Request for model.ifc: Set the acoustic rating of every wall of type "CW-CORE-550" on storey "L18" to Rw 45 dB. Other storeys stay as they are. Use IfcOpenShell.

First a look at what the model holds.

```python
import ifcopenshell
import ifcopenshell.util.element

model = ifcopenshell.open("model.ifc")
print(model.schema)
storey = next(s for s in model.by_type("IfcBuildingStorey") if s.Name == "L18")
walls = [e for e in ifcopenshell.util.element.get_decomposition(storey) if e.is_a("IfcWall")]
seen = {}
for e in walls:
    element_type = ifcopenshell.util.element.get_type(e)
    key = (element_type.Name if element_type != e and element_type else None, ifcopenshell.util.element.get_pset(e, "Pset_WallCommon", "AcousticRating"))
    seen[key] = seen.get(key, 0) + 1
for (name, value), count in sorted(seen.items(), key=str):
    print(count, "x", name, "|", value)
```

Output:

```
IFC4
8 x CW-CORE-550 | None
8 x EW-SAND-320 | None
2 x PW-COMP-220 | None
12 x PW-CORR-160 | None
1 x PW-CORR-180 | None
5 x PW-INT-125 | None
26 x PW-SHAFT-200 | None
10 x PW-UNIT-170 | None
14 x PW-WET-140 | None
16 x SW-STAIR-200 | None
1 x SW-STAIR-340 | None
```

```python
import ifcopenshell
import ifcopenshell.api.pset
import ifcopenshell.util.element

model = ifcopenshell.open("model.ifc")

storey = next(s for s in model.by_type("IfcBuildingStorey") if s.Name == "L18")
walls = [e for e in ifcopenshell.util.element.get_decomposition(storey) if e.is_a("IfcWall")]

count = 0
for e in walls:
    element_type = ifcopenshell.util.element.get_type(e)
    if element_type in (None, e) or element_type.Name != "CW-CORE-550":
        continue
    found = ifcopenshell.util.element.get_pset(e, "Pset_WallCommon", should_inherit=False)
    if found:
        pset = model.by_id(found["id"])
        if len(ifcopenshell.util.element.get_elements_by_pset(pset)) > 1:
            pset = ifcopenshell.api.pset.unshare_pset(model, products=[e], pset=pset)[0]
    else:
        pset = ifcopenshell.api.pset.add_pset(model, product=e, name="Pset_WallCommon")
    ifcopenshell.api.pset.edit_pset(model, pset=pset, properties={"AcousticRating": "Rw 45 dB"})
    count += 1

print(count, "walls updated")

model.write("model_edited.ifc")
```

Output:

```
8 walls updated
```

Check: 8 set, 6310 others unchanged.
